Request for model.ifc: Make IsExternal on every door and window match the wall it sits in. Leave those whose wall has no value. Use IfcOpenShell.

First a look at what the model holds.

```python
import ifcopenshell
import ifcopenshell.util.element

model = ifcopenshell.open("model.ifc")
print(model.schema)
seen = {}
for e in model.by_type("IfcDoor") + model.by_type("IfcWindow"):
    if not e.FillsVoids:
        continue
    host = e.FillsVoids[0].RelatingOpeningElement.VoidsElements[0].RelatingBuildingElement
    own = ifcopenshell.util.element.get_pset(e, f"Pset_{e.is_a()[3:].removesuffix('StandardCase')}Common", "IsExternal")
    wall = ifcopenshell.util.element.get_pset(host, "Pset_WallCommon", "IsExternal")
    seen[e.is_a(), own, wall] = seen.get((e.is_a(), own, wall), 0) + 1
for (cls, own, wall), count in sorted(seen.items(), key=str):
    print(count, cls, "IsExternal:", own, "| host wall:", wall)
```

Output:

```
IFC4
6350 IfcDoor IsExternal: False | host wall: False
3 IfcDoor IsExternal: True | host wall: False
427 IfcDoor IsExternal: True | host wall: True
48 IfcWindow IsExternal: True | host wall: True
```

```python
import ifcopenshell
import ifcopenshell.api.pset
import ifcopenshell.util.element

model = ifcopenshell.open("model.ifc")

count = 0
for ifc_class, pset_name in (("IfcDoor", "Pset_DoorCommon"), ("IfcWindow", "Pset_WindowCommon")):
    for e in model.by_type(ifc_class):
        if not e.FillsVoids:
            continue
        host = e.FillsVoids[0].RelatingOpeningElement.VoidsElements[0].RelatingBuildingElement
        external = ifcopenshell.util.element.get_pset(host, "Pset_WallCommon", "IsExternal")
        if external is None or ifcopenshell.util.element.get_pset(e, pset_name, "IsExternal") == external:
            continue
        pset = ifcopenshell.api.pset.add_pset(model, product=e, name=pset_name)
        ifcopenshell.api.pset.edit_pset(model, pset=pset, properties={"IsExternal": external})
        count += 1

print(count, "updated")

model.write("model_updated.ifc")
```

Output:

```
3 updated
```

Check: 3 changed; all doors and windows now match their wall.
